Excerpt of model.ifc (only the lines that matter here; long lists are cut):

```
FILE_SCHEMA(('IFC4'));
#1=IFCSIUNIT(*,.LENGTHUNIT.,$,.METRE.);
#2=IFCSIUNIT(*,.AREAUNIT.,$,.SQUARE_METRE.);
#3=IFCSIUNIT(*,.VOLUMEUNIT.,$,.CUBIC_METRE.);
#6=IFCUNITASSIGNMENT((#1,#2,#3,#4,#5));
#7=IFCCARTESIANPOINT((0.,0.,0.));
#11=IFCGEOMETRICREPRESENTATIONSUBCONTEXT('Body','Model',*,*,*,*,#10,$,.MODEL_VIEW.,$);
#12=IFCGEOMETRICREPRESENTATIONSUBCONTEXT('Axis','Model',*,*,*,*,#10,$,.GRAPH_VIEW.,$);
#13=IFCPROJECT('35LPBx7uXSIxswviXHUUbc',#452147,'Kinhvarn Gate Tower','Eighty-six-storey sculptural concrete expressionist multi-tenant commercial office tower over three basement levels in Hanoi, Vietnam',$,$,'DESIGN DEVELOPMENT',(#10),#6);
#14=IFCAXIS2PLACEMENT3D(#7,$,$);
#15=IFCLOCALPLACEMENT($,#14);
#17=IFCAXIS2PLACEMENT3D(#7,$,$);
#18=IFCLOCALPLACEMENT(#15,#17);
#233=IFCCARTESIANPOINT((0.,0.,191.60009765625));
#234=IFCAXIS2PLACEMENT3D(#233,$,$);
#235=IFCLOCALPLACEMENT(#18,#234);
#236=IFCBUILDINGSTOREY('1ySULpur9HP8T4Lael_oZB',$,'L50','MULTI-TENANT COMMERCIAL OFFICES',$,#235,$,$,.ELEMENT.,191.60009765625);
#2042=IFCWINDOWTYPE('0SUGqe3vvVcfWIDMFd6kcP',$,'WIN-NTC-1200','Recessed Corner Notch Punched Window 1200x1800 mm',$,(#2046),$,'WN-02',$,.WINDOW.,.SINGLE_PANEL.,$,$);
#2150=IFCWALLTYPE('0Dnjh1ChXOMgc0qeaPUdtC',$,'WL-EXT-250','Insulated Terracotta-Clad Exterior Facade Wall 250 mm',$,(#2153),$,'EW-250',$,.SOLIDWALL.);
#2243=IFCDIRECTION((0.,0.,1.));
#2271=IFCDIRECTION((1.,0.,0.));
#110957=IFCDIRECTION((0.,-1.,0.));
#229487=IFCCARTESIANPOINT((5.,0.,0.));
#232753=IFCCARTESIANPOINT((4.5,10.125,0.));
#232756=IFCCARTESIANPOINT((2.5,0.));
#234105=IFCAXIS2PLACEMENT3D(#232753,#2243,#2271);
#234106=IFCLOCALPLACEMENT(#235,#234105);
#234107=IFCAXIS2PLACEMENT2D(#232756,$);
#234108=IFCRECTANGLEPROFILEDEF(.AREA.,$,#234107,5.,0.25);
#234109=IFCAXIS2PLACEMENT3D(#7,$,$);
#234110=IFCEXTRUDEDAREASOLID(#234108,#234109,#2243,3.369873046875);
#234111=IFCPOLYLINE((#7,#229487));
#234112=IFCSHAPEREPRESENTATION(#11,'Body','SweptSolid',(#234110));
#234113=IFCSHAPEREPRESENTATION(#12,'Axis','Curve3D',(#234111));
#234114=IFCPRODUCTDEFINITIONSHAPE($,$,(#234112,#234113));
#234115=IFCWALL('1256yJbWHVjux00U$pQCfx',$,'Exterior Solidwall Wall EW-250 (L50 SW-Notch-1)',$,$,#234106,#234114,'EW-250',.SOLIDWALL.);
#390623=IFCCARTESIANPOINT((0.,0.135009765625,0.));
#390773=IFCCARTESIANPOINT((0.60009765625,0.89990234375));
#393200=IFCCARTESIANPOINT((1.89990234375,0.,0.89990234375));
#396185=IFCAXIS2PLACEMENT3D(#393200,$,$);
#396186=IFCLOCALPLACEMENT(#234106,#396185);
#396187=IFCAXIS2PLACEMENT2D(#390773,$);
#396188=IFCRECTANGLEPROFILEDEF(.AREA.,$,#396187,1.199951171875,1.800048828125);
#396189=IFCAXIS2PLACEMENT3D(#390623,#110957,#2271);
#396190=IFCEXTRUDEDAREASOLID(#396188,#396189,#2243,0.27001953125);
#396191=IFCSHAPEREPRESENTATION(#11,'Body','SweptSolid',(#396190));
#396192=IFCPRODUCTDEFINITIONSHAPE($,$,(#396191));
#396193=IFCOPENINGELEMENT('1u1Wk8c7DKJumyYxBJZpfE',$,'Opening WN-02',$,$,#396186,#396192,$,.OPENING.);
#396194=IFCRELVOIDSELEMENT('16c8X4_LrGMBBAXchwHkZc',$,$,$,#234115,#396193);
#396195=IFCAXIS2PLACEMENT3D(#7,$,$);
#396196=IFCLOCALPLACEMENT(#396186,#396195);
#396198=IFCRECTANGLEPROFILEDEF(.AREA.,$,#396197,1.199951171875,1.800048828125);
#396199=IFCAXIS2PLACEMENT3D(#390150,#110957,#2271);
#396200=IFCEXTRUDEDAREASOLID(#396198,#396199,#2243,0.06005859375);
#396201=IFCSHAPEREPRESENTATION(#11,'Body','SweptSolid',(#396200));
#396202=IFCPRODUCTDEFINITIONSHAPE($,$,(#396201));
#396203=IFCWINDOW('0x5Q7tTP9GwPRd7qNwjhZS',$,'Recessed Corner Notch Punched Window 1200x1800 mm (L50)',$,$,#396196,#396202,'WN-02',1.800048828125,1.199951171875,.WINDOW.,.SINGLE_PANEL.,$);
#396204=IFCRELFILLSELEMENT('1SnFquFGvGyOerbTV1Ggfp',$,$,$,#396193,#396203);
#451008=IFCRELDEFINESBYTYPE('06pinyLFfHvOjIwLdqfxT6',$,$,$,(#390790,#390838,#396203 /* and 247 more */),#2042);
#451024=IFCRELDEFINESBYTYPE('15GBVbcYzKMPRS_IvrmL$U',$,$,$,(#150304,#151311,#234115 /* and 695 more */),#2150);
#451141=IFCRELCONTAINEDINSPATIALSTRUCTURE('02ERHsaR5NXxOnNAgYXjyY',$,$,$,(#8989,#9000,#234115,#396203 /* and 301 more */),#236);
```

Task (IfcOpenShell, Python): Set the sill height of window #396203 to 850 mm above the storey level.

```python
import numpy as np
import ifcopenshell
import ifcopenshell.api.geometry
import ifcopenshell.geom
import ifcopenshell.util.element
import ifcopenshell.util.placement
import ifcopenshell.util.shape
import ifcopenshell.util.unit

model = ifcopenshell.open("model.ifc")
unit_scale = ifcopenshell.util.unit.calculate_unit_scale(model)

window = model.by_id(396203)
opening = window.FillsVoids[0].RelatingOpeningElement
storey = ifcopenshell.util.element.get_container(window, ifc_class="IfcBuildingStorey")
level = ifcopenshell.util.placement.get_local_placement(storey.ObjectPlacement)[2, 3]

# The opening's origin need not be at the sill, so measure its lowest point.
shape = ifcopenshell.geom.create_shape(ifcopenshell.geom.settings(), opening)
bottom = ifcopenshell.util.shape.get_shape_bottom_elevation(shape, shape.geometry) / unit_scale
dz = level + 0.85 / unit_scale - bottom

shift = np.array([0.0, 0.0, dz])
# The window is placed relative to its opening, so it follows when the opening moves.
matrix = ifcopenshell.util.placement.get_local_placement(opening.ObjectPlacement)
matrix[:3, 3] += shift
ifcopenshell.api.geometry.edit_object_placement(
    model, product=opening, matrix=matrix, is_si=False, should_transform_children=True
)

print(f"moved by {dz * unit_scale:+.3f} m")

model.write("model_edited.ifc")
```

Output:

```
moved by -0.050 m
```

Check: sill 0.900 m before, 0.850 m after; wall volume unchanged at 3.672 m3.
